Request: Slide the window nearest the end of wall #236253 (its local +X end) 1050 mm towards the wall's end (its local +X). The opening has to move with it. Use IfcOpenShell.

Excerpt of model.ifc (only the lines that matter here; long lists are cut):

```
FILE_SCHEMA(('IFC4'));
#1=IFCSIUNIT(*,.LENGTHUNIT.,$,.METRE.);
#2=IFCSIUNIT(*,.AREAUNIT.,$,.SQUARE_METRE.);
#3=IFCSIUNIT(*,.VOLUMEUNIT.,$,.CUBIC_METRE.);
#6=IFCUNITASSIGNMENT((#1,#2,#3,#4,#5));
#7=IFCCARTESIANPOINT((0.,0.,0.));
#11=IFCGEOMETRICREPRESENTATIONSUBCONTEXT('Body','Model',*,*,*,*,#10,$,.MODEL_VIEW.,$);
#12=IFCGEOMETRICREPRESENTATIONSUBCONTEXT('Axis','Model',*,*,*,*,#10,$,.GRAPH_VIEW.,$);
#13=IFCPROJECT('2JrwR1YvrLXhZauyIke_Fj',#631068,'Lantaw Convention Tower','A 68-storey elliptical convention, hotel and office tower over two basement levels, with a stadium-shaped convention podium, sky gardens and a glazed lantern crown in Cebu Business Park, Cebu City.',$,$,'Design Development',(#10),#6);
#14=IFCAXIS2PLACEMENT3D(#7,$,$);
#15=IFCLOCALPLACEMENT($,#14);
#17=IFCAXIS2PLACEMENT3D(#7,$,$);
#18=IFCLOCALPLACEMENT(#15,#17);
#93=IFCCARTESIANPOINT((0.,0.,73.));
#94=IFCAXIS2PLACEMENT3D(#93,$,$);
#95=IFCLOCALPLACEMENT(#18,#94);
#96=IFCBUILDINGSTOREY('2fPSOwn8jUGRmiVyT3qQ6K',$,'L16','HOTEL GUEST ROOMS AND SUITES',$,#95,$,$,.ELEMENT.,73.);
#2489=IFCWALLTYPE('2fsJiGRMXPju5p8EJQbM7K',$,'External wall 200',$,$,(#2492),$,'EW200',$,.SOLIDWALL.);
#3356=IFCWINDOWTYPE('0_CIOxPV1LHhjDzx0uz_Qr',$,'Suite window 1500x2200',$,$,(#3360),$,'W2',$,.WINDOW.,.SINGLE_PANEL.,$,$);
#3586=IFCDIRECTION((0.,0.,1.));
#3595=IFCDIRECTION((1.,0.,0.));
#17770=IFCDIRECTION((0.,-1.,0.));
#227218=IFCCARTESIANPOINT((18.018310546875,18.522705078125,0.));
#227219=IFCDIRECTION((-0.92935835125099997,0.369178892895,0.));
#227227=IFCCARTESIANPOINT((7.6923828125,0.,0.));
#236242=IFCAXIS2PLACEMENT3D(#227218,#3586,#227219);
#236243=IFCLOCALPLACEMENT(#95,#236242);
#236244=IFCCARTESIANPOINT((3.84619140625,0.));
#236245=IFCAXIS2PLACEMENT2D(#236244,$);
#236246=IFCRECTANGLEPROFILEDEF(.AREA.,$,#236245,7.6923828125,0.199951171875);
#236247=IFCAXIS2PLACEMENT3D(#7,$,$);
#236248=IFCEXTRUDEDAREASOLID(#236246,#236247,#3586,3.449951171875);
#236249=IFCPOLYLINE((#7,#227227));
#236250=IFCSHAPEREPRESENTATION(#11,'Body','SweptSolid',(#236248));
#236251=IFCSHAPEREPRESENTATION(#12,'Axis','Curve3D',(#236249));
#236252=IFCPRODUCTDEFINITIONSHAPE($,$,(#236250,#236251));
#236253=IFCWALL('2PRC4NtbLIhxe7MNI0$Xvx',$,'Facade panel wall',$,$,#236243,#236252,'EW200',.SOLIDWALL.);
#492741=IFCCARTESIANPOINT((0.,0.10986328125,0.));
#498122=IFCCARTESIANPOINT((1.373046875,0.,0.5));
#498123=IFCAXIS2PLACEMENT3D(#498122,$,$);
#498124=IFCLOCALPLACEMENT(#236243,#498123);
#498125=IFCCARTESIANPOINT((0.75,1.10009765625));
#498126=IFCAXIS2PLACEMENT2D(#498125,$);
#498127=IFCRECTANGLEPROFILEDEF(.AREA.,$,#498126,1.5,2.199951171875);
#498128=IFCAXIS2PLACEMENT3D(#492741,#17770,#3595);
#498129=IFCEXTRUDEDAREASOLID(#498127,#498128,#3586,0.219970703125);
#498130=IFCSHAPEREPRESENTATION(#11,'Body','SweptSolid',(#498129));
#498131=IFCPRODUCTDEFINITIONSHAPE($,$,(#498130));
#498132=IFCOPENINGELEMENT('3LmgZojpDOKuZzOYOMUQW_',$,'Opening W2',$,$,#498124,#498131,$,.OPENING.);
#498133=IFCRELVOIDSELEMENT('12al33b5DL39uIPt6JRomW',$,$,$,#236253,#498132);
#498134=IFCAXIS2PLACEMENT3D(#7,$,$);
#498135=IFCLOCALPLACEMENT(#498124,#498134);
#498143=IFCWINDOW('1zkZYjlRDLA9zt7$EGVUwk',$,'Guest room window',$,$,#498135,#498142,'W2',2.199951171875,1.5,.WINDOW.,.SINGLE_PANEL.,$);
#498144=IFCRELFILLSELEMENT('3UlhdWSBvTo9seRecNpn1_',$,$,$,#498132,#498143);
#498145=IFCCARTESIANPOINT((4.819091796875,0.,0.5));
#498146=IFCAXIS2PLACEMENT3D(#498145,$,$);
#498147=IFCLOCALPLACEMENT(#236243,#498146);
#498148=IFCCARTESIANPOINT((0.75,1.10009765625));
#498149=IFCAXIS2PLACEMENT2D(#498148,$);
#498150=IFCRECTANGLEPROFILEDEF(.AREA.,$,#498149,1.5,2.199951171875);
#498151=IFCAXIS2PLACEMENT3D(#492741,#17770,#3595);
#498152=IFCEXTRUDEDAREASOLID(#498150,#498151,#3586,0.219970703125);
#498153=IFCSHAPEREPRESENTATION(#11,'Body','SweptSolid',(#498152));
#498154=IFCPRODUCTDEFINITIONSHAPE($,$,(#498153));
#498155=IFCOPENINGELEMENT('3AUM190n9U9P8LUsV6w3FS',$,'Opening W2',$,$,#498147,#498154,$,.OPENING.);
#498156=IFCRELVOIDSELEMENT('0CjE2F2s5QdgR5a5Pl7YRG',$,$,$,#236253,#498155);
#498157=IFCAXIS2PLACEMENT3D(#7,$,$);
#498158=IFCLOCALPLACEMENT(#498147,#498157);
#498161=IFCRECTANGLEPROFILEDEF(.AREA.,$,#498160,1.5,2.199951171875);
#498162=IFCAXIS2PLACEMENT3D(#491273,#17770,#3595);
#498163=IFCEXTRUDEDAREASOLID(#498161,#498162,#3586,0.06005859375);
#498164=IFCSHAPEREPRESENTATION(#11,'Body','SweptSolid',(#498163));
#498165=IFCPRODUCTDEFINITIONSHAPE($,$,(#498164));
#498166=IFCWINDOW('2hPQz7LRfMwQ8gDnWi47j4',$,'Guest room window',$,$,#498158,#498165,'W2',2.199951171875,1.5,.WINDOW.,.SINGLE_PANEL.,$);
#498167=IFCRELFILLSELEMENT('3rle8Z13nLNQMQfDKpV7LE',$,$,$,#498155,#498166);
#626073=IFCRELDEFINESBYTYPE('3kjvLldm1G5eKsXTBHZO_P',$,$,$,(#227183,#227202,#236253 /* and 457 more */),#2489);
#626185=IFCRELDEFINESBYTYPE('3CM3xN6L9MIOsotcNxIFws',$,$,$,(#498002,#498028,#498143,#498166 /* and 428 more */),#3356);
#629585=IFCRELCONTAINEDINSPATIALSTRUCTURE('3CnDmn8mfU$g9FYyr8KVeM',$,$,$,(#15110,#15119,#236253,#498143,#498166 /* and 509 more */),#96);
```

```python
import ifcopenshell
import ifcopenshell.api.geometry
import ifcopenshell.util.placement

model = ifcopenshell.open("model.ifc")

window = model.by_guid("2hPQz7LRfMwQ8gDnWi47j4")
opening = window.FillsVoids[0].RelatingOpeningElement
wall = opening.VoidsElements[0].RelatingBuildingElement

wall_matrix = ifcopenshell.util.placement.get_local_placement(wall.ObjectPlacement)
shift = wall_matrix[:3, 0] * 1.05
before = ifcopenshell.util.placement.get_local_placement(window.ObjectPlacement)[:3, 3].copy()

# The window is placed relative to its opening, so it follows when the opening moves.
matrix = ifcopenshell.util.placement.get_local_placement(opening.ObjectPlacement)
matrix[:3, 3] += shift
ifcopenshell.api.geometry.edit_object_placement(
    model, product=opening, matrix=matrix, is_si=False, should_transform_children=True
)

after = ifcopenshell.util.placement.get_local_placement(window.ObjectPlacement)[:3, 3]
print("window moved by", (after - before).round(3) + 0.0)

model.write("model_rev.ifc")
```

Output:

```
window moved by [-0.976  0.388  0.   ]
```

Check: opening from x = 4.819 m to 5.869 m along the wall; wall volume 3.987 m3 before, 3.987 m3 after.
